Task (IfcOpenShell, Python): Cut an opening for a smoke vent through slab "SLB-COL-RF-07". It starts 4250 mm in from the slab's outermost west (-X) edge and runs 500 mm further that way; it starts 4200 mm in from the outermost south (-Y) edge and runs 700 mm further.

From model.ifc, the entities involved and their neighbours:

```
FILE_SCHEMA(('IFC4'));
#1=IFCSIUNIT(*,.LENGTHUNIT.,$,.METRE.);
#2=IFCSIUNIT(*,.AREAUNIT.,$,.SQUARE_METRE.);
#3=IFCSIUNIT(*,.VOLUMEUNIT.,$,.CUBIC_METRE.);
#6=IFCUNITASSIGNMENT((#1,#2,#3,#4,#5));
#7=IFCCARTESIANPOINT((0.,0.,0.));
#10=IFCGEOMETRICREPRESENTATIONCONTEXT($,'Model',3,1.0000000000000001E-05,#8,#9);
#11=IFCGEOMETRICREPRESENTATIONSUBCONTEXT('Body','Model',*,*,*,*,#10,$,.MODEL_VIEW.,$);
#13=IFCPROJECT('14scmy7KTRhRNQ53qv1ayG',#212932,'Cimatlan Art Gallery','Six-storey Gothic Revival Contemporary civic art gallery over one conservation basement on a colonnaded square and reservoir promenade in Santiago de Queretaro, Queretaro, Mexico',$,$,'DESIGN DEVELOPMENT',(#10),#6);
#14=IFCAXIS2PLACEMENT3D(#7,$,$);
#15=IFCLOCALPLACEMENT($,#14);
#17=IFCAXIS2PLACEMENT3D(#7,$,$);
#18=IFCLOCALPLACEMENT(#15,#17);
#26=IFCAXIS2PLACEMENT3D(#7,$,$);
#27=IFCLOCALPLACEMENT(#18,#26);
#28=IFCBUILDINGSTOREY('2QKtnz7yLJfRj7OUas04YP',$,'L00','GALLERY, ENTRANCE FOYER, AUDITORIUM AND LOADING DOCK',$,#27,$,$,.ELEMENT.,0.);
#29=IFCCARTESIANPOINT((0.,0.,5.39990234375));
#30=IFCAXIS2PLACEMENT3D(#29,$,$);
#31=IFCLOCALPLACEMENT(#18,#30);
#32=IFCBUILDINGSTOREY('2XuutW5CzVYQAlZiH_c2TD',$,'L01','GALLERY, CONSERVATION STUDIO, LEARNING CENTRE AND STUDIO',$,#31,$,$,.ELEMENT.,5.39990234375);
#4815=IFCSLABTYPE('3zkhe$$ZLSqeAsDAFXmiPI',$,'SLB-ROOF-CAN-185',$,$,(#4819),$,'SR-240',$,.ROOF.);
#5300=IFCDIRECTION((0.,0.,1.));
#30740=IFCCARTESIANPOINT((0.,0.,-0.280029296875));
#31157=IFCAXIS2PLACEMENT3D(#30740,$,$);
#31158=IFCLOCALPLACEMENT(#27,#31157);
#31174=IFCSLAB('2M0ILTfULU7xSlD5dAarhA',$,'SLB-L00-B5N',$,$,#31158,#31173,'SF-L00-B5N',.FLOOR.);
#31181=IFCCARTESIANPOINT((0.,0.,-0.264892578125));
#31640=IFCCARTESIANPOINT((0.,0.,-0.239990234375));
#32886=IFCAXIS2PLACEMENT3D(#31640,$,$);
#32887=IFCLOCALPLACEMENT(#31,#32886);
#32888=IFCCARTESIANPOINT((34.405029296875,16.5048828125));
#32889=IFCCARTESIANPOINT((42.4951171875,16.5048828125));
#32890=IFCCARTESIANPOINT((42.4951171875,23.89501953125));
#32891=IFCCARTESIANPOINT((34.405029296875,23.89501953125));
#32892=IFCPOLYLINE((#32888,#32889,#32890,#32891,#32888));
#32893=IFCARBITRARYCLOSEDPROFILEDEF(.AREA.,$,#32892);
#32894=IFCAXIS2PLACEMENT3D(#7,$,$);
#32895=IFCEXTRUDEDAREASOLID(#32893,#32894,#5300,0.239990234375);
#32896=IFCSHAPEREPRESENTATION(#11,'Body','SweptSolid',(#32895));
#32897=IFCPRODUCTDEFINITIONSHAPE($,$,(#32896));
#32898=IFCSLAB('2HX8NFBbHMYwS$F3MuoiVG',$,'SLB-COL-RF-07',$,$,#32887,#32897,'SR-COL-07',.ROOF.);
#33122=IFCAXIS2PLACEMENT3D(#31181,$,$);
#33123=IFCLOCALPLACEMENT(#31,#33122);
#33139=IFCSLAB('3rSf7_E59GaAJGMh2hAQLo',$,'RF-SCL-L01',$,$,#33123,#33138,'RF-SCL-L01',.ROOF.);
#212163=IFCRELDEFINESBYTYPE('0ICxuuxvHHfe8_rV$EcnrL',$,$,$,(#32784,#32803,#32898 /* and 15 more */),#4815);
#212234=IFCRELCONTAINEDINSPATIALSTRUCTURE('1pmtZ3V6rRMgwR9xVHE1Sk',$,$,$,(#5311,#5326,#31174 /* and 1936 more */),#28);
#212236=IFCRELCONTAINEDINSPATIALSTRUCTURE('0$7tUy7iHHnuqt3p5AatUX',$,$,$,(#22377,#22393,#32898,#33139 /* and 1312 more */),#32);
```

```python
import numpy as np
import ifcopenshell
import ifcopenshell.api.feature
import ifcopenshell.api.geometry
import ifcopenshell.api.root
import ifcopenshell.geom
import ifcopenshell.util.placement
import ifcopenshell.util.representation
import ifcopenshell.util.shape
import ifcopenshell.util.unit

model = ifcopenshell.open("model.ifc")
unit_scale = ifcopenshell.util.unit.calculate_unit_scale(model)
settings = ifcopenshell.geom.settings()


def volume(element):
    """Net volume in cubic metres, openings subtracted."""
    shape = ifcopenshell.geom.create_shape(settings, element)
    return ifcopenshell.util.shape.get_volume(shape.geometry)


slab = model.by_id(32898)
before = volume(slab)

# Extent in the slab's own axes, in metres. The edges named are its -X and -Y sides.
slab_shape = ifcopenshell.geom.create_shape(settings, slab)
vertices = ifcopenshell.util.shape.get_vertices(slab_shape.geometry)
x_min, y_min, bottom = vertices.min(axis=0)
top = vertices[:, 2].max()

opening = ifcopenshell.api.root.create_entity(model, ifc_class="IfcOpeningElement", name="Smoke vent opening", predefined_type="OPENING")
context = ifcopenshell.util.representation.get_context(model, "Model", "Body", "MODEL_VIEW")
width, depth = 0.5, 0.7
outline = [(0.0, 0.0), (width, 0.0), (width, depth), (0.0, depth), (0.0, 0.0)]
# Overshoot both faces by 50 mm so the cut is clean.
shape = ifcopenshell.api.geometry.add_slab_representation(
    model, context=context, depth=top - bottom + 0.1, polyline=outline
)
ifcopenshell.api.geometry.assign_representation(model, product=opening, representation=shape)

matrix = ifcopenshell.util.placement.get_local_placement(slab.ObjectPlacement)
matrix[:, 3] = matrix @ np.append(np.array([x_min + 4.25, y_min + 4.2, bottom - 0.05]) / unit_scale, 1.0)
ifcopenshell.api.geometry.edit_object_placement(model, product=opening, matrix=matrix, is_si=False)
ifcopenshell.api.feature.add_feature(model, feature=opening, element=slab)

after = volume(slab)

print(f"slab volume {before:.3f} -> {after:.3f} m3")

model.write("model-out.ifc")
```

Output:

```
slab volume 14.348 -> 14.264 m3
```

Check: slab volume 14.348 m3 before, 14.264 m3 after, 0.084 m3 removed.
